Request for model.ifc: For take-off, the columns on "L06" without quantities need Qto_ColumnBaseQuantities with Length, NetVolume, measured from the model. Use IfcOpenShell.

First a look at what the model holds.

```python
import ifcopenshell
import ifcopenshell.util.element
import ifcopenshell.util.unit

model = ifcopenshell.open("model.ifc")
print(model.schema)
for unit_type in ("LENGTHUNIT", "AREAUNIT", "VOLUMEUNIT"):
    print(unit_type, ifcopenshell.util.unit.calculate_unit_scale(model, unit_type))
storey = next(s for s in model.by_type("IfcBuildingStorey") if s.Name == "L06")
columns = [e for e in ifcopenshell.util.element.get_decomposition(storey) if e.is_a("IfcColumn")]
for e in sorted(columns, key=lambda e: e.id()):
    print(e.id(), e.is_a(), e.Name, list(ifcopenshell.util.element.get_psets(e, qtos_only=True)), sep=" | ")
```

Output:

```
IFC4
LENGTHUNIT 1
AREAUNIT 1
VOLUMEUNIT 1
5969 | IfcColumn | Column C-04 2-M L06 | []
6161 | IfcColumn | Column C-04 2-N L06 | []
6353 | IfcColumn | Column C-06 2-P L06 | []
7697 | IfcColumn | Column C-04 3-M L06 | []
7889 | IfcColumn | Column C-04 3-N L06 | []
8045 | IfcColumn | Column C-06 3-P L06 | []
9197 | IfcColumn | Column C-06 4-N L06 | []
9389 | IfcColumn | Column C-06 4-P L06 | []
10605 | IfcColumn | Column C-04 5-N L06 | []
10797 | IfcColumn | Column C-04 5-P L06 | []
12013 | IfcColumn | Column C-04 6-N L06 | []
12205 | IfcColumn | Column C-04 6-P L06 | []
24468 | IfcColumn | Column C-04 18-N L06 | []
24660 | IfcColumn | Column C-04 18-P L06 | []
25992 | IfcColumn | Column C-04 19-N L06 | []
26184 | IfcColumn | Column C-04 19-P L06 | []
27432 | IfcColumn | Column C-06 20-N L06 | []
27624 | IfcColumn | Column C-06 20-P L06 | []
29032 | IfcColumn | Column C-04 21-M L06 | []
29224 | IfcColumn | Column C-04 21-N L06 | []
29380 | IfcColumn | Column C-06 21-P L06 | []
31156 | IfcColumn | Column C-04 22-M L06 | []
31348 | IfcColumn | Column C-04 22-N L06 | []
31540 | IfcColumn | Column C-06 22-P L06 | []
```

```python
import ifcopenshell
import ifcopenshell.api.pset
import ifcopenshell.geom
import ifcopenshell.util.element
import ifcopenshell.util.shape
import ifcopenshell.util.unit

model = ifcopenshell.open("model.ifc")
unit_scale = ifcopenshell.util.unit.calculate_unit_scale(model)
volume_scale = ifcopenshell.util.unit.calculate_unit_scale(model, "VOLUMEUNIT")
settings = ifcopenshell.geom.settings()

storey = next(s for s in model.by_type("IfcBuildingStorey") if s.Name == "L06")
columns = [e for e in ifcopenshell.util.element.get_decomposition(storey) if e.is_a("IfcColumn")]

for e in sorted(columns, key=lambda e: e.id()):
    if ifcopenshell.util.element.get_psets(e, qtos_only=True, should_inherit=False):
        continue
    # Geometry comes back in metres, in the element's own axes.
    shape = ifcopenshell.geom.create_shape(settings, e)
    values = {
        "Length": ifcopenshell.util.shape.get_z(shape.geometry) / unit_scale,
        "NetVolume": ifcopenshell.util.shape.get_volume(shape.geometry) / volume_scale,
    }
    qto = ifcopenshell.api.pset.add_qto(model, product=e, name="Qto_ColumnBaseQuantities")
    ifcopenshell.api.pset.edit_qto(model, qto=qto, properties=values)
    print(e.id(), {k: round(v, 3) for k, v in values.items()})

model.write("model_updated.ifc")
```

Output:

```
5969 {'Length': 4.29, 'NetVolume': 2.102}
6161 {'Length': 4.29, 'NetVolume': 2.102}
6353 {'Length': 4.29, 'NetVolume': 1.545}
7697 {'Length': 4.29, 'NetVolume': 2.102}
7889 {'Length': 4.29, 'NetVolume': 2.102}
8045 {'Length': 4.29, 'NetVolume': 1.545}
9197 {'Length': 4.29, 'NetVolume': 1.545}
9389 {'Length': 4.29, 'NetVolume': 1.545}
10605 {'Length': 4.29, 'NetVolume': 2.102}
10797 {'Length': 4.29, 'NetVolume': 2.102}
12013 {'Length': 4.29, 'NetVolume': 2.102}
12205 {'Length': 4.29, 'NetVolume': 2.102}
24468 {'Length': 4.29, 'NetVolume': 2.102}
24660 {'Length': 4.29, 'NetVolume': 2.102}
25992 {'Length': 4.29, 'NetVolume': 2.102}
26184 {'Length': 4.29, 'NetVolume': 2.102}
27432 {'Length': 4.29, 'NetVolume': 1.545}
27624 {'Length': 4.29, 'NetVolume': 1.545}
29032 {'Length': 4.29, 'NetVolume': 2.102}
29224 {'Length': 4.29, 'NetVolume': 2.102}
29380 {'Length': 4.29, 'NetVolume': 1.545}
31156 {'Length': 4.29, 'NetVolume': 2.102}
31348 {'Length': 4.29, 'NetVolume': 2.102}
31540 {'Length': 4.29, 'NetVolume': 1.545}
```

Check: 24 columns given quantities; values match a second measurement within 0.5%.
